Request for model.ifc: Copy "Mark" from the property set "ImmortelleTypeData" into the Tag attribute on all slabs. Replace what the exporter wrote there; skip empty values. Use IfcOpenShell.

First a look at what the model holds.

```python
import ifcopenshell
import ifcopenshell.util.element

model = ifcopenshell.open("model.ifc")
print(model.schema)
slabs = model.by_type("IfcSlab")
print(len(slabs), "slabs")
for e in slabs[:8]:
    source = ifcopenshell.util.element.get_pset(e, "ImmortelleTypeData", "Mark")
    target = e.Tag
    print(e.id(), repr(source), repr(target), sep=" | ")
```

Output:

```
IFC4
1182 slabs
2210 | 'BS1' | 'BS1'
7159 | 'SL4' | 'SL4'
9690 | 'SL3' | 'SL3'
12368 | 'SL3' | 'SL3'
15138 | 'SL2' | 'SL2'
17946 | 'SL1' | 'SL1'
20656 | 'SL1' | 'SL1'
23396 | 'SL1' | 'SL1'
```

```python
import ifcopenshell
import ifcopenshell.util.element

model = ifcopenshell.open("model.ifc")

count = 0
for e in model.by_type("IfcSlab"):
    value = ifcopenshell.util.element.get_pset(e, "ImmortelleTypeData", "Mark")
    current = e.Tag
    if not value or not value.strip() or current == value:
        continue
    e.Tag = value
    count += 1

print(count, "slabs updated")

model.write("model_rev.ifc")
```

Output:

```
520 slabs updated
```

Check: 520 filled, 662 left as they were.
